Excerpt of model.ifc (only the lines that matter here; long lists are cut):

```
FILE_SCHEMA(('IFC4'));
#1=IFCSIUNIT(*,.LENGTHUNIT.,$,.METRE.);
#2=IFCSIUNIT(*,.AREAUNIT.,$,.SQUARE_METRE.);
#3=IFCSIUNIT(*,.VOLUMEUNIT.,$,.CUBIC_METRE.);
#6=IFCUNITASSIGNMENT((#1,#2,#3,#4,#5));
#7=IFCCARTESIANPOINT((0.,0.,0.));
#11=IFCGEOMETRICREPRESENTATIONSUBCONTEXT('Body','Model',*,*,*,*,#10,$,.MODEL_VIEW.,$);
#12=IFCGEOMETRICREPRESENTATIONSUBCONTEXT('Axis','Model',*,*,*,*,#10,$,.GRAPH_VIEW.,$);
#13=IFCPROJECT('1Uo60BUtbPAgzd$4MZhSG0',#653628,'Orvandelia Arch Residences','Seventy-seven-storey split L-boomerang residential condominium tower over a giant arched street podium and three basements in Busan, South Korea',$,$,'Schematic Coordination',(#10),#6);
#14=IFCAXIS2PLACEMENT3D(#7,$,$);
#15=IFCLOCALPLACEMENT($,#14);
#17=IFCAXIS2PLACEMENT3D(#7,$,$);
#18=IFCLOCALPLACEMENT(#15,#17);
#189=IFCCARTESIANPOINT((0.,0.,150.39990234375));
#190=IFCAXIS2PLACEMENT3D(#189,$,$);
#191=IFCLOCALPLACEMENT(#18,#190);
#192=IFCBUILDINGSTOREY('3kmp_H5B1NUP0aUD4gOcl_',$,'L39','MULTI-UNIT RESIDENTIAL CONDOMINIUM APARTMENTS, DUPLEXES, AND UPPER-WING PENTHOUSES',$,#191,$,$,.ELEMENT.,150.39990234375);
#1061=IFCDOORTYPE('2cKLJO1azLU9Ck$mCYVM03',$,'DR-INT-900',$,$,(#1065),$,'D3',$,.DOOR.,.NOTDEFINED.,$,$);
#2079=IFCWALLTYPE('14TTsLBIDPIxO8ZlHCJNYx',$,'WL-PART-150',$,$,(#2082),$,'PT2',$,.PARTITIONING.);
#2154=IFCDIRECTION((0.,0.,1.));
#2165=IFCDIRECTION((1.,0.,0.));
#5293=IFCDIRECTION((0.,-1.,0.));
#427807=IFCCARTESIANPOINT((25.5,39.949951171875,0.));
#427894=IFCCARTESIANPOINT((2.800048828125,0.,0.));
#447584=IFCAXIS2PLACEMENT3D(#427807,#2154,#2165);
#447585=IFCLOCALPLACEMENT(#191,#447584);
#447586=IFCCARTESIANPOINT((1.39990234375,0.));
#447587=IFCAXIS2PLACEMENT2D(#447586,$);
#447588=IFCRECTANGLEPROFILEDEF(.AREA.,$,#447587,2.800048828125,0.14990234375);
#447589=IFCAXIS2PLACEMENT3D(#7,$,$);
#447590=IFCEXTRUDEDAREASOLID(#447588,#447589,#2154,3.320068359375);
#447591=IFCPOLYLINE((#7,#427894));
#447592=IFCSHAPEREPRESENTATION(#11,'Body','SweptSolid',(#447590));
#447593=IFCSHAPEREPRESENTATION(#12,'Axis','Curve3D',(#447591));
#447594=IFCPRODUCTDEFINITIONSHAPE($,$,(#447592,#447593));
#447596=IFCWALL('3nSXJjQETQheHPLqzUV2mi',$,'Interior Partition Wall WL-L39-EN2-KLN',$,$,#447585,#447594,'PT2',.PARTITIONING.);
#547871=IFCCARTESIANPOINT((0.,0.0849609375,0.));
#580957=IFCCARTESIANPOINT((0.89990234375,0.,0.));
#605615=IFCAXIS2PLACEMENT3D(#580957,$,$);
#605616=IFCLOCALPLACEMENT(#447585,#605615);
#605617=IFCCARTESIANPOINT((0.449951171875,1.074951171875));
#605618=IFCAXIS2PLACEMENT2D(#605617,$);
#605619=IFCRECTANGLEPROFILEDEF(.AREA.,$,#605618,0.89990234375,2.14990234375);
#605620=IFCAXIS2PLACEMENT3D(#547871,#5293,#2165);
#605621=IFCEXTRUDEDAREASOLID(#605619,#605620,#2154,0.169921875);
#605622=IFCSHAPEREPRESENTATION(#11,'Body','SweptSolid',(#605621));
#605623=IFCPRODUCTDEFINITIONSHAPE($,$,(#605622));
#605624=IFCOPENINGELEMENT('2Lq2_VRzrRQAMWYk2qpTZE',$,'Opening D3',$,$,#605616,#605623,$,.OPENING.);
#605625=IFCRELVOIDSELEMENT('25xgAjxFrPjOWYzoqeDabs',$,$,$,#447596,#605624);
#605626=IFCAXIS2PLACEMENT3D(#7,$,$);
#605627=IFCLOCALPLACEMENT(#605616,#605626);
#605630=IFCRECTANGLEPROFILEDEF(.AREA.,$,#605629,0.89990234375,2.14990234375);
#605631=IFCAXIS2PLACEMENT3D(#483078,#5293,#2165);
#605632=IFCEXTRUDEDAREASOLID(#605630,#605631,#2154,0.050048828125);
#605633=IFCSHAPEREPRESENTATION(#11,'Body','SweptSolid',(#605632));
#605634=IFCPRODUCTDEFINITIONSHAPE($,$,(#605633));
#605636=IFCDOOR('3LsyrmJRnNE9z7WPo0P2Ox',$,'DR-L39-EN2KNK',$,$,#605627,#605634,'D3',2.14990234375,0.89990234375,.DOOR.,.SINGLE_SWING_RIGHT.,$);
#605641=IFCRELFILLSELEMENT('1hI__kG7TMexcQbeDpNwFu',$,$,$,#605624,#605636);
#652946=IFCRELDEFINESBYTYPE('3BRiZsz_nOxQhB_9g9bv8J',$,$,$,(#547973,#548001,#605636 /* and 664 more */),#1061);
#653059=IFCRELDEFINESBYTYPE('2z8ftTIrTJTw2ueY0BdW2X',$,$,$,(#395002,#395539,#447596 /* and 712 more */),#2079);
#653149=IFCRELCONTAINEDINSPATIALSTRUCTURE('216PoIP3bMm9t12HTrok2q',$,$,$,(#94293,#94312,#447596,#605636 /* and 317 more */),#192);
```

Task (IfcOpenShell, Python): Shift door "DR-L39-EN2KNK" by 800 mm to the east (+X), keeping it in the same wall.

```python
import ifcopenshell
import ifcopenshell.api.geometry
import ifcopenshell.util.placement
import ifcopenshell.util.unit

model = ifcopenshell.open("model.ifc")
unit_scale = ifcopenshell.util.unit.calculate_unit_scale(model)

door = model.by_guid("3LsyrmJRnNE9z7WPo0P2Ox")
opening = door.FillsVoids[0].RelatingOpeningElement
wall = opening.VoidsElements[0].RelatingBuildingElement

wall_matrix = ifcopenshell.util.placement.get_local_placement(wall.ObjectPlacement)
shift = wall_matrix[:3, 0] * 0.8 / unit_scale
before = ifcopenshell.util.placement.get_local_placement(door.ObjectPlacement)[:3, 3].copy()

# The door is placed relative to its opening, so it follows when the opening moves.
matrix = ifcopenshell.util.placement.get_local_placement(opening.ObjectPlacement)
matrix[:3, 3] += shift
ifcopenshell.api.geometry.edit_object_placement(
    model, product=opening, matrix=matrix, is_si=False, should_transform_children=True
)

after = ifcopenshell.util.placement.get_local_placement(door.ObjectPlacement)[:3, 3]
print("door moved by", (after - before).round(3) + 0.0)

model.write("model_edited.ifc")
```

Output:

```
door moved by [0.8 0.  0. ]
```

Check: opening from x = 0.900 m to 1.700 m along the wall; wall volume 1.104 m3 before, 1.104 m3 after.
